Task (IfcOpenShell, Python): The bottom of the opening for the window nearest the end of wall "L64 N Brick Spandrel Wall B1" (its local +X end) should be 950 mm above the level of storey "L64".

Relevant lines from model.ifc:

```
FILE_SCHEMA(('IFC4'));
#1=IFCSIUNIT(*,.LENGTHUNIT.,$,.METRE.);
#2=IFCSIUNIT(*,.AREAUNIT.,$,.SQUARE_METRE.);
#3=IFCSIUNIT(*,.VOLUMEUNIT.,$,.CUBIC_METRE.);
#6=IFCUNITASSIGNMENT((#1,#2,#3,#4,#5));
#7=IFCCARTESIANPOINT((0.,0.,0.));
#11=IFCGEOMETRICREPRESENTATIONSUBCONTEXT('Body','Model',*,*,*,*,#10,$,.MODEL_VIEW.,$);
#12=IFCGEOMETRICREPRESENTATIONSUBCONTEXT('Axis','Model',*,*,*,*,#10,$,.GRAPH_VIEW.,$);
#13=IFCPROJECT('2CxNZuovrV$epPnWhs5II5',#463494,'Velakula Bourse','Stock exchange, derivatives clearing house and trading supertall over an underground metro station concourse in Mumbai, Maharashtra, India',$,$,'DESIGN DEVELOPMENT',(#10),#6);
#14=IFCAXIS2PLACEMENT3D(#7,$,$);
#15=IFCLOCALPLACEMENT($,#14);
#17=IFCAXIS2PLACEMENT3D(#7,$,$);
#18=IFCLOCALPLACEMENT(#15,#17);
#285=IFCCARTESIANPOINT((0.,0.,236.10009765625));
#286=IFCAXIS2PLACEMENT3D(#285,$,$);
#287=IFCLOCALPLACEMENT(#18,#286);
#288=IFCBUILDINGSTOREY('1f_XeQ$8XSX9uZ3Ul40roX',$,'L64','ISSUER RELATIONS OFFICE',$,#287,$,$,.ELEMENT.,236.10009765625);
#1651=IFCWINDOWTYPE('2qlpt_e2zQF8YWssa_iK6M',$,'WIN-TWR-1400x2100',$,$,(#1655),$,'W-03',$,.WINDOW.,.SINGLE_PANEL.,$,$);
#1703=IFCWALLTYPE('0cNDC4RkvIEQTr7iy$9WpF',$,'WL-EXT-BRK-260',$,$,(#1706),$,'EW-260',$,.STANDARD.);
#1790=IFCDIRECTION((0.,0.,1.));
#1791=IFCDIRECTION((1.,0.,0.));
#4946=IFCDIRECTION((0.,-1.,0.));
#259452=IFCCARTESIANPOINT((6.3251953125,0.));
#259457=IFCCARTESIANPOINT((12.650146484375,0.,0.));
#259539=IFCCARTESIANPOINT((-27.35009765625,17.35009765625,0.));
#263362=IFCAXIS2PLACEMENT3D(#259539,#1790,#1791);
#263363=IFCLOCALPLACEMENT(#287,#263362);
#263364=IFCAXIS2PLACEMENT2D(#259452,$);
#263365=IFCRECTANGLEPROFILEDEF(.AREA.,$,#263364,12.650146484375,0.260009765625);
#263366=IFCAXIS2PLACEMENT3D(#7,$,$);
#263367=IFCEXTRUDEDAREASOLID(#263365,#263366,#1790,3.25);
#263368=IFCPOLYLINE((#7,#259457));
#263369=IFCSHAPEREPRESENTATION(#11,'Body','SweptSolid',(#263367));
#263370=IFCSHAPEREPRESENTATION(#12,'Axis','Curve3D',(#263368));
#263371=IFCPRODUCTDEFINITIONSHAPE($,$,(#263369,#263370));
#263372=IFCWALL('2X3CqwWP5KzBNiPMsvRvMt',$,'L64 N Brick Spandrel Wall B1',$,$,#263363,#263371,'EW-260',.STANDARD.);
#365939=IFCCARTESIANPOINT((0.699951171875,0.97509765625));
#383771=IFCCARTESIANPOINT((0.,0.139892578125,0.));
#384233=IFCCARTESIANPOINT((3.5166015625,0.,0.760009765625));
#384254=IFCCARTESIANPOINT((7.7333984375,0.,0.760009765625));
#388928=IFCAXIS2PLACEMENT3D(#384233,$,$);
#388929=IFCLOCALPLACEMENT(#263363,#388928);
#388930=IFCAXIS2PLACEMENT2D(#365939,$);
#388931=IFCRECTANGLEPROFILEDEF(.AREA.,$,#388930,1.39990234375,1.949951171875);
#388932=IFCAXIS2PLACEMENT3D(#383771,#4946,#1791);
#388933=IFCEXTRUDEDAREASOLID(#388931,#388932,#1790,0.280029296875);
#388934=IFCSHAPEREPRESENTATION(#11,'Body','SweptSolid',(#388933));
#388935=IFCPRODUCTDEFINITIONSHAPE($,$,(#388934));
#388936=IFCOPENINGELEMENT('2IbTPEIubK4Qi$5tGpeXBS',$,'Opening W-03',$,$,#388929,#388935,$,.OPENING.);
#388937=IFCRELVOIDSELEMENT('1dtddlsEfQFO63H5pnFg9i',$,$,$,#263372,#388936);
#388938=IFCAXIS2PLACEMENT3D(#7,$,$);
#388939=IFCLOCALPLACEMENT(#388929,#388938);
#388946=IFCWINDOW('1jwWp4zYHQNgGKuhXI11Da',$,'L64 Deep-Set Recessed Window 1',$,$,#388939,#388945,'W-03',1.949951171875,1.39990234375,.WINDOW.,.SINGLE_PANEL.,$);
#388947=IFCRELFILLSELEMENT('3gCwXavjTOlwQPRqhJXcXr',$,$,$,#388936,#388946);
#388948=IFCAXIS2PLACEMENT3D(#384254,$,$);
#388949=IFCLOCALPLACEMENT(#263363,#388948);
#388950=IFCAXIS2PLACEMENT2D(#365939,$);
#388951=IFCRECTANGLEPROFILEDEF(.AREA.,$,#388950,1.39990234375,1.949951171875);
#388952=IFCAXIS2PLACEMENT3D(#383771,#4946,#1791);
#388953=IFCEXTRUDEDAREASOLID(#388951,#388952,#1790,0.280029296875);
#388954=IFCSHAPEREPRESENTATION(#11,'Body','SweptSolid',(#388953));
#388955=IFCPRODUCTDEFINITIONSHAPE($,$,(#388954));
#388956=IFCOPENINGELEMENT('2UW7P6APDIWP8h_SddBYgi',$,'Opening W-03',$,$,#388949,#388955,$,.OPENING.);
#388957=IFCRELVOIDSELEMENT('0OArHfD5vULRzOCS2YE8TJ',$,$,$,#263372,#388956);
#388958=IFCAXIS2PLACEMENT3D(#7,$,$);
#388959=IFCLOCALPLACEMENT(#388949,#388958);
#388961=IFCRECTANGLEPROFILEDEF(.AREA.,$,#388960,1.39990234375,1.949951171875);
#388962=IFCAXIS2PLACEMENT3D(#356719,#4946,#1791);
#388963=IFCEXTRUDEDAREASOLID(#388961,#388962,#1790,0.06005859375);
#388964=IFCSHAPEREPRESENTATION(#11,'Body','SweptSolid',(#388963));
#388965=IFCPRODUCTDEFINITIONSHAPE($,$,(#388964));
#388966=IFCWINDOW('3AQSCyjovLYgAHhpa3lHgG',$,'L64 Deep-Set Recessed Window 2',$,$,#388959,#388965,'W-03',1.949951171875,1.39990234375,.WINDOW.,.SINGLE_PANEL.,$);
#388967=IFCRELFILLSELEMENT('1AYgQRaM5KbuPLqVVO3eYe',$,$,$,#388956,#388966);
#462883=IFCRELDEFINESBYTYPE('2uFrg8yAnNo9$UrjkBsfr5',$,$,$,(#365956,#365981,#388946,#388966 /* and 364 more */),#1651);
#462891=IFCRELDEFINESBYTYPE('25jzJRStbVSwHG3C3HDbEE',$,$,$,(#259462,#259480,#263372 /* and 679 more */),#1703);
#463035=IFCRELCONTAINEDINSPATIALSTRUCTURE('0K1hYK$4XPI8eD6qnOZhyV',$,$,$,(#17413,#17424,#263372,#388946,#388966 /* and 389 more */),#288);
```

```python
import numpy as np
import ifcopenshell
import ifcopenshell.api.geometry
import ifcopenshell.geom
import ifcopenshell.util.element
import ifcopenshell.util.placement
import ifcopenshell.util.shape
import ifcopenshell.util.unit

model = ifcopenshell.open("model.ifc")
unit_scale = ifcopenshell.util.unit.calculate_unit_scale(model)

window = model.by_guid("3AQSCyjovLYgAHhpa3lHgG")
opening = window.FillsVoids[0].RelatingOpeningElement
storey = ifcopenshell.util.element.get_container(window, ifc_class="IfcBuildingStorey")
level = ifcopenshell.util.placement.get_local_placement(storey.ObjectPlacement)[2, 3]

# The opening's origin need not be at the sill, so measure its lowest point.
shape = ifcopenshell.geom.create_shape(ifcopenshell.geom.settings(), opening)
bottom = ifcopenshell.util.shape.get_shape_bottom_elevation(shape, shape.geometry) / unit_scale
dz = level + 0.95 / unit_scale - bottom

shift = np.array([0.0, 0.0, dz])
# The window is placed relative to its opening, so it follows when the opening moves.
matrix = ifcopenshell.util.placement.get_local_placement(opening.ObjectPlacement)
matrix[:3, 3] += shift
ifcopenshell.api.geometry.edit_object_placement(
    model, product=opening, matrix=matrix, is_si=False, should_transform_children=True
)

print(f"moved by {dz * unit_scale:+.3f} m")

model.write("model_v2.ifc")
```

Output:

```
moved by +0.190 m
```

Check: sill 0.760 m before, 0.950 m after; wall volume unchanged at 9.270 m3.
